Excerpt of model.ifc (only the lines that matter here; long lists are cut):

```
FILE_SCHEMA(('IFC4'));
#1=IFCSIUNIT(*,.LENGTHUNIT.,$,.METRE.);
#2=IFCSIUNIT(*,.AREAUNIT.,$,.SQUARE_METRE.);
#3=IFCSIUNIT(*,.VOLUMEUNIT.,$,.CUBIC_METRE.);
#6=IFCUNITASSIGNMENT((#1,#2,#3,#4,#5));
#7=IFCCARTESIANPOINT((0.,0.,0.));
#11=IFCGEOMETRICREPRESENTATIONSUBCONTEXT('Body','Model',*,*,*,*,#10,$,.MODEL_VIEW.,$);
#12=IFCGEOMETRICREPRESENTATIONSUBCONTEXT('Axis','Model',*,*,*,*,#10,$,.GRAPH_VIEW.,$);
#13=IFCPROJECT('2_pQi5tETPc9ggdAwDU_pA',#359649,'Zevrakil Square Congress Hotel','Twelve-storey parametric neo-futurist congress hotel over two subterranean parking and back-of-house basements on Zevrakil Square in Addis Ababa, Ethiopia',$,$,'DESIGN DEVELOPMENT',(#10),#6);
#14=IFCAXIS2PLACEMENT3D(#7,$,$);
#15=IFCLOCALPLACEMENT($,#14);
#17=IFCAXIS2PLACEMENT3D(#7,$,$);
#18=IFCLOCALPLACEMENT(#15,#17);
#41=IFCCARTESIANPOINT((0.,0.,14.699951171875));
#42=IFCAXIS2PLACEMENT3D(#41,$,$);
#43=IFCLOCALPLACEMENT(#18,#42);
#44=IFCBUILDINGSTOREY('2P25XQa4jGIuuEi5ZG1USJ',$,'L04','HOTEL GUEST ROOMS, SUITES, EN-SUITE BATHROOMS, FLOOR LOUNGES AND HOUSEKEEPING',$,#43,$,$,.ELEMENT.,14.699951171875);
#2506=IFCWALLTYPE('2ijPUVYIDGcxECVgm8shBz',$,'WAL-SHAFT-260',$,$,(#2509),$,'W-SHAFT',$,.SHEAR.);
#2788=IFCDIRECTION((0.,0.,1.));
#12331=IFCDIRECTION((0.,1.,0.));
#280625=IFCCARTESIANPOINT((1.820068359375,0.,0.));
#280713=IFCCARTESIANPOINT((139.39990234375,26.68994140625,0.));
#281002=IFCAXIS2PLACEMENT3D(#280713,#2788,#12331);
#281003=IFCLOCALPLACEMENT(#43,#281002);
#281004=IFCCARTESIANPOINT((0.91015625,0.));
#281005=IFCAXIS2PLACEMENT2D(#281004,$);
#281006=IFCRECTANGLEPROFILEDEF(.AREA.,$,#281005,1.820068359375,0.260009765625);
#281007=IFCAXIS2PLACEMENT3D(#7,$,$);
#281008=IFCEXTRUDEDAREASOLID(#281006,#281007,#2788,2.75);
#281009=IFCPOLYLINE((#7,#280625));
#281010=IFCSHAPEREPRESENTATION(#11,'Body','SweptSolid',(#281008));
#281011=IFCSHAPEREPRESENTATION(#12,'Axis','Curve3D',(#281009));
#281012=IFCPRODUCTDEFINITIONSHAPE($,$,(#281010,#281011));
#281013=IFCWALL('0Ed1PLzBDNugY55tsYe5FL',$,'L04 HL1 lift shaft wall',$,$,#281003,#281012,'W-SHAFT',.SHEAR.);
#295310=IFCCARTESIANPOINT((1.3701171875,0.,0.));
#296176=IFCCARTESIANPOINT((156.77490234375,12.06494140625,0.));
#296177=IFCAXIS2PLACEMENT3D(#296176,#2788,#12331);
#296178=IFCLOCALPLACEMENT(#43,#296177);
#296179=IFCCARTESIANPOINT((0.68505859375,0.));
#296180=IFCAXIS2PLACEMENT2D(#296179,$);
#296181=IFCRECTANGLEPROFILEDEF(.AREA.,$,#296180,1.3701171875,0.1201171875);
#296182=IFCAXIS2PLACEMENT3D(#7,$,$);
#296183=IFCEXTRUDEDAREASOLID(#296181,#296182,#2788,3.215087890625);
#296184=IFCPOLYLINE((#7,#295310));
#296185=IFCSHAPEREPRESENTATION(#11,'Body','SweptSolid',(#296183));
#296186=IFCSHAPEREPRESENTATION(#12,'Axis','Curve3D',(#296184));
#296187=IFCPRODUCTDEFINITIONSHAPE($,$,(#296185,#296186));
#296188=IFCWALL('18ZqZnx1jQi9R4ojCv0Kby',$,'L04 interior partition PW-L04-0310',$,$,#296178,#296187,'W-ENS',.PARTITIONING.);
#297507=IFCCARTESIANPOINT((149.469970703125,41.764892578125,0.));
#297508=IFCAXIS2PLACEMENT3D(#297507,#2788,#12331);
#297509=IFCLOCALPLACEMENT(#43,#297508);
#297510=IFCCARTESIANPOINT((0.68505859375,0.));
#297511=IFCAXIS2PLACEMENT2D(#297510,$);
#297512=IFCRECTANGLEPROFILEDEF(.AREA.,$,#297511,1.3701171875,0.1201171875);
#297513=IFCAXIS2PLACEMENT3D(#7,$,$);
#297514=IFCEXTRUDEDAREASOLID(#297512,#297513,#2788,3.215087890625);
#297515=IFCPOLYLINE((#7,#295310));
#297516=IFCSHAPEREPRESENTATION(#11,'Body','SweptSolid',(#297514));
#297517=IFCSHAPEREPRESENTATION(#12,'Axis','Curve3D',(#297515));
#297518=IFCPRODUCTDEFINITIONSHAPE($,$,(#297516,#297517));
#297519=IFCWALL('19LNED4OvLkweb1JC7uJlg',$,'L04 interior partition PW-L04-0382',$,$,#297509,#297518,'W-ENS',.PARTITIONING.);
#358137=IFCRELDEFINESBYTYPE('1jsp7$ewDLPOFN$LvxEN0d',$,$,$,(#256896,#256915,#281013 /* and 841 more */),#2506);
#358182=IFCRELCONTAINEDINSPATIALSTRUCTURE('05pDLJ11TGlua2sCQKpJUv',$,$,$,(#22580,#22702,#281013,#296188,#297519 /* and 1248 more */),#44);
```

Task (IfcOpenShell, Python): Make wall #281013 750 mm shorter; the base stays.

```python
import ifcopenshell
import ifcopenshell.geom
import ifcopenshell.util.representation
import ifcopenshell.util.shape

model = ifcopenshell.open("model.ifc")
settings = ifcopenshell.geom.settings()


def volume(element):
    """Net volume in cubic metres, openings subtracted."""
    shape = ifcopenshell.geom.create_shape(settings, element)
    return ifcopenshell.util.shape.get_volume(shape.geometry)


wall = model.by_guid("0Ed1PLzBDNugY55tsYe5FL")
before = volume(wall)

body = ifcopenshell.util.representation.get_representation(wall, "Model", "Body")
solid = body.Items[0]
old_height = solid.Depth
solid.Depth -= 0.75
after = volume(wall)

print(f"height {old_height:g} -> {solid.Depth:g}, volume {before:.3f} -> {after:.3f} m3")

model.write("model_edited.ifc")
```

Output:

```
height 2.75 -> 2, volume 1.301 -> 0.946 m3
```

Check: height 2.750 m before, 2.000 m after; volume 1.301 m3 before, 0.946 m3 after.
